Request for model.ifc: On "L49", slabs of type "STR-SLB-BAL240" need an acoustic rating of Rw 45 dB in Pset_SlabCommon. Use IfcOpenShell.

First a look at what the model holds.

```python
import ifcopenshell
import ifcopenshell.util.element

model = ifcopenshell.open("model.ifc")
print(model.schema)
storey = next(s for s in model.by_type("IfcBuildingStorey") if s.Name == "L49")
slabs = [e for e in ifcopenshell.util.element.get_decomposition(storey) if e.is_a("IfcSlab")]
seen = {}
for e in slabs:
    element_type = ifcopenshell.util.element.get_type(e)
    key = (element_type.Name if element_type != e and element_type else None, ifcopenshell.util.element.get_pset(e, "Pset_SlabCommon", "AcousticRating"))
    seen[key] = seen.get(key, 0) + 1
for (name, value), count in sorted(seen.items(), key=str):
    print(count, "x", name, "|", value)
```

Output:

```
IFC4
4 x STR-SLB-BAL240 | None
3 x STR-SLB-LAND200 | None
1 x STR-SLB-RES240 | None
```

```python
import ifcopenshell
import ifcopenshell.api.pset
import ifcopenshell.util.element

model = ifcopenshell.open("model.ifc")

storey = next(s for s in model.by_type("IfcBuildingStorey") if s.Name == "L49")
slabs = [e for e in ifcopenshell.util.element.get_decomposition(storey) if e.is_a("IfcSlab")]

count = 0
for e in slabs:
    element_type = ifcopenshell.util.element.get_type(e)
    if element_type in (None, e) or element_type.Name != "STR-SLB-BAL240":
        continue
    found = ifcopenshell.util.element.get_pset(e, "Pset_SlabCommon", should_inherit=False)
    if found:
        pset = model.by_id(found["id"])
        if len(ifcopenshell.util.element.get_elements_by_pset(pset)) > 1:
            pset = ifcopenshell.api.pset.unshare_pset(model, products=[e], pset=pset)[0]
    else:
        pset = ifcopenshell.api.pset.add_pset(model, product=e, name="Pset_SlabCommon")
    ifcopenshell.api.pset.edit_pset(model, pset=pset, properties={"AcousticRating": "Rw 45 dB"})
    count += 1

print(count, "slabs updated")

model.write("model_v2.ifc")
```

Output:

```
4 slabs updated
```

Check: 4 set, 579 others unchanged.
